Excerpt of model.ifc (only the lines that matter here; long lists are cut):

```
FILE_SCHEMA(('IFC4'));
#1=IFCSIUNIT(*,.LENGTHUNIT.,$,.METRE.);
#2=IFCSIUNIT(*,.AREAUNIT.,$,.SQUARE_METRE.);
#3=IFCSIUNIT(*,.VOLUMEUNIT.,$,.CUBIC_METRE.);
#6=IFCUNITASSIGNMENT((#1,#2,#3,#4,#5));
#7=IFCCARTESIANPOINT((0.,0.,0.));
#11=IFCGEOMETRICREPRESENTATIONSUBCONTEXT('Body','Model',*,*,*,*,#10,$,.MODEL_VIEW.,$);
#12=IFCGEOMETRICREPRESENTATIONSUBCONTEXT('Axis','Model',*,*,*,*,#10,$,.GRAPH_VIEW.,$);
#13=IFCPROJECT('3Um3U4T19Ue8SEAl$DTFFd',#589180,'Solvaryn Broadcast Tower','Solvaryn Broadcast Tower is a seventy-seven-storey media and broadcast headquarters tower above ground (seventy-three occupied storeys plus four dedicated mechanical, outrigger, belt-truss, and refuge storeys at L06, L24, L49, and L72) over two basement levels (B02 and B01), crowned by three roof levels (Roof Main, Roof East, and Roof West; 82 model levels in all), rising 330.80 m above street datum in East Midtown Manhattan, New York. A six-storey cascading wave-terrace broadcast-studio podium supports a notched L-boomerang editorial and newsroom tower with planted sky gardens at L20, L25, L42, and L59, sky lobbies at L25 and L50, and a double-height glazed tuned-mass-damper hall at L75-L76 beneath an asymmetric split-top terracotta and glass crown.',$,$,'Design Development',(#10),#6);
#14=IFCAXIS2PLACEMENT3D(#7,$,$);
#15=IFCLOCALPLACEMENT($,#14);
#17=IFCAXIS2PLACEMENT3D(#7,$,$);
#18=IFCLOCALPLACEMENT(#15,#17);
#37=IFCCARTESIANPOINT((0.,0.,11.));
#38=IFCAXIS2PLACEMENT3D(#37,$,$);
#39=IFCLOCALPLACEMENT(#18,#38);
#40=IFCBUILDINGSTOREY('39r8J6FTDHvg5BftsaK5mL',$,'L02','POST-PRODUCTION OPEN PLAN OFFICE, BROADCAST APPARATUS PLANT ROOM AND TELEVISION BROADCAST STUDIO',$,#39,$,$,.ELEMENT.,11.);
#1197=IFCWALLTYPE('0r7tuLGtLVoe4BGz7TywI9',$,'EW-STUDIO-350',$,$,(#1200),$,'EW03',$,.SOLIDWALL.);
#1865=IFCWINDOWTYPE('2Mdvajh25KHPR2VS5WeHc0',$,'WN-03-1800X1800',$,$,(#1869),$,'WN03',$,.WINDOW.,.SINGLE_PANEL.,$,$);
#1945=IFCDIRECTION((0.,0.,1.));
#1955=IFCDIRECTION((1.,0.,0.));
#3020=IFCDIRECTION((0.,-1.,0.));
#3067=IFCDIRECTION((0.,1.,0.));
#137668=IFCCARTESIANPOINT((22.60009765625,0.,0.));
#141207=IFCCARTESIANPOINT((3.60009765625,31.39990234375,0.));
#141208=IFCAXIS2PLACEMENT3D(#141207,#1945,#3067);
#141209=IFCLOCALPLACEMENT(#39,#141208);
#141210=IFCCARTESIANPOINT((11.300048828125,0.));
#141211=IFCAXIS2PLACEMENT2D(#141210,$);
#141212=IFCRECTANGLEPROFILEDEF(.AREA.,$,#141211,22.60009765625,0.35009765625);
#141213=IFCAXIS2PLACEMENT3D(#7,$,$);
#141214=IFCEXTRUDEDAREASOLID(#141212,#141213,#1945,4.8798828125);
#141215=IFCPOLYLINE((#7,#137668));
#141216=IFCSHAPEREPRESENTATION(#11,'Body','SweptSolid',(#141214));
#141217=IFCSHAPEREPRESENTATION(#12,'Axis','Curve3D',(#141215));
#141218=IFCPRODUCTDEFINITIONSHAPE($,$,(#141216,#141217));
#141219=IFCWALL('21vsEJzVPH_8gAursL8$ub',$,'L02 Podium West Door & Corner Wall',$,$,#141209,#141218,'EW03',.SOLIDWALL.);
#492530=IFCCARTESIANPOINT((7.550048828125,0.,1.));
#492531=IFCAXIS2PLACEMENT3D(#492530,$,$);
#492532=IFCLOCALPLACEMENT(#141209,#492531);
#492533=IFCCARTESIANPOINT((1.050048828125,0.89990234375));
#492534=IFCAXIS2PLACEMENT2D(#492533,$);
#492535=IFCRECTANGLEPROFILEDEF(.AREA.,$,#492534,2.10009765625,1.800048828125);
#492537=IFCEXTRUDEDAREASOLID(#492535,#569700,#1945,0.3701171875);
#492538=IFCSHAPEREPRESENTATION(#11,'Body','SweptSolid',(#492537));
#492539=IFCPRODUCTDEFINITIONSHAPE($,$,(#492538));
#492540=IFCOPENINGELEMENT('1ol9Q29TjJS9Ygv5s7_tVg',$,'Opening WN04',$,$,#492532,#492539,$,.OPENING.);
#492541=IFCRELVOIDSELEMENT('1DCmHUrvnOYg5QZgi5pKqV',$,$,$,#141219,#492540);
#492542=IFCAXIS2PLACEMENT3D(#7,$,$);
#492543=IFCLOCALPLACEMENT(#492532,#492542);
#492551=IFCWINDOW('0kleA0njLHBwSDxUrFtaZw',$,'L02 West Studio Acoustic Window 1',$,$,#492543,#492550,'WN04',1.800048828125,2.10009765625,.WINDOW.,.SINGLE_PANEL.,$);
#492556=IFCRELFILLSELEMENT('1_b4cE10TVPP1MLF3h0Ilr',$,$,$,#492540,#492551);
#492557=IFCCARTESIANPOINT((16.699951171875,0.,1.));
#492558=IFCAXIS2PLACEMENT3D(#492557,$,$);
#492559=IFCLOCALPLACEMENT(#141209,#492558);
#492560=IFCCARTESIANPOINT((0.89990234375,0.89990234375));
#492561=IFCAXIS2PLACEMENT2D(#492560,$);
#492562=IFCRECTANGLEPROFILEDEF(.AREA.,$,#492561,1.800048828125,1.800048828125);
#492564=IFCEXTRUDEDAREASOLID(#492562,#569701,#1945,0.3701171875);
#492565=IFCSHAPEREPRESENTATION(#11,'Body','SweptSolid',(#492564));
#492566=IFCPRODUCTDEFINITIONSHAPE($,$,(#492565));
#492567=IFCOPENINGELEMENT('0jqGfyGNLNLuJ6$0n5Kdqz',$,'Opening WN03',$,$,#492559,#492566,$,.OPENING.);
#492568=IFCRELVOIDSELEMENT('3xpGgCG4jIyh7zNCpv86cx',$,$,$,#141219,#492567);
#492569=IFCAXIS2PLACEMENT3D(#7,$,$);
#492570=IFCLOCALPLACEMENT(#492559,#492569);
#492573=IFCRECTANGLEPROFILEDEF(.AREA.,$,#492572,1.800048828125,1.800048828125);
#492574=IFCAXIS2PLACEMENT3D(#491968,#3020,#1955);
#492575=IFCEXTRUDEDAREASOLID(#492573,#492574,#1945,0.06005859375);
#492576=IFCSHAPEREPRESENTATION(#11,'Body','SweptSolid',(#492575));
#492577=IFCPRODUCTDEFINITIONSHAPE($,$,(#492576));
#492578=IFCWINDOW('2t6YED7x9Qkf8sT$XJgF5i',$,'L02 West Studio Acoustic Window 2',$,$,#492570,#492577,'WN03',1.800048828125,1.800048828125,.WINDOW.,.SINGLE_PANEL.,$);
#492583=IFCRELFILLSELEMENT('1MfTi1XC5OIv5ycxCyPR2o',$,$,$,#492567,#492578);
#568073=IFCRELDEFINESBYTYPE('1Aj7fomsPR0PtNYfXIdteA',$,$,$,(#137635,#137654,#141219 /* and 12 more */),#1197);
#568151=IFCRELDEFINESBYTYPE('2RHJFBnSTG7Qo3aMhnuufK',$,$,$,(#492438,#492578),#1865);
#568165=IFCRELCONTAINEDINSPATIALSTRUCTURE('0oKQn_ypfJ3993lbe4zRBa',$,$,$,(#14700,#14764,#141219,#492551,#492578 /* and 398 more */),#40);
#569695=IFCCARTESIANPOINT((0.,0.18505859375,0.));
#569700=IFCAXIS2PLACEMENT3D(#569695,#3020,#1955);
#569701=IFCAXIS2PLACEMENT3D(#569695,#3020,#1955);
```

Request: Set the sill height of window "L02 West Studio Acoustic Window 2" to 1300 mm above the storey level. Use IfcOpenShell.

```python
import numpy as np
import ifcopenshell
import ifcopenshell.api.geometry
import ifcopenshell.geom
import ifcopenshell.util.element
import ifcopenshell.util.placement
import ifcopenshell.util.shape
import ifcopenshell.util.unit

model = ifcopenshell.open("model.ifc")
unit_scale = ifcopenshell.util.unit.calculate_unit_scale(model)

window = model.by_guid("2t6YED7x9Qkf8sT$XJgF5i")
opening = window.FillsVoids[0].RelatingOpeningElement
storey = ifcopenshell.util.element.get_container(window, ifc_class="IfcBuildingStorey")
level = ifcopenshell.util.placement.get_local_placement(storey.ObjectPlacement)[2, 3]

# The opening's origin need not be at the sill, so measure its lowest point.
shape = ifcopenshell.geom.create_shape(ifcopenshell.geom.settings(), opening)
bottom = ifcopenshell.util.shape.get_shape_bottom_elevation(shape, shape.geometry) / unit_scale
dz = level + 1.3 / unit_scale - bottom

shift = np.array([0.0, 0.0, dz])
# The window is placed relative to its opening, so it follows when the opening moves.
matrix = ifcopenshell.util.placement.get_local_placement(opening.ObjectPlacement)
matrix[:3, 3] += shift
ifcopenshell.api.geometry.edit_object_placement(
    model, product=opening, matrix=matrix, is_si=False, should_transform_children=True
)

print(f"moved by {dz * unit_scale:+.3f} m")

model.write("model-out.ifc")
```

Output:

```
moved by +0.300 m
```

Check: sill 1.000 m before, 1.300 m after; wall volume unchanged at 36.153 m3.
